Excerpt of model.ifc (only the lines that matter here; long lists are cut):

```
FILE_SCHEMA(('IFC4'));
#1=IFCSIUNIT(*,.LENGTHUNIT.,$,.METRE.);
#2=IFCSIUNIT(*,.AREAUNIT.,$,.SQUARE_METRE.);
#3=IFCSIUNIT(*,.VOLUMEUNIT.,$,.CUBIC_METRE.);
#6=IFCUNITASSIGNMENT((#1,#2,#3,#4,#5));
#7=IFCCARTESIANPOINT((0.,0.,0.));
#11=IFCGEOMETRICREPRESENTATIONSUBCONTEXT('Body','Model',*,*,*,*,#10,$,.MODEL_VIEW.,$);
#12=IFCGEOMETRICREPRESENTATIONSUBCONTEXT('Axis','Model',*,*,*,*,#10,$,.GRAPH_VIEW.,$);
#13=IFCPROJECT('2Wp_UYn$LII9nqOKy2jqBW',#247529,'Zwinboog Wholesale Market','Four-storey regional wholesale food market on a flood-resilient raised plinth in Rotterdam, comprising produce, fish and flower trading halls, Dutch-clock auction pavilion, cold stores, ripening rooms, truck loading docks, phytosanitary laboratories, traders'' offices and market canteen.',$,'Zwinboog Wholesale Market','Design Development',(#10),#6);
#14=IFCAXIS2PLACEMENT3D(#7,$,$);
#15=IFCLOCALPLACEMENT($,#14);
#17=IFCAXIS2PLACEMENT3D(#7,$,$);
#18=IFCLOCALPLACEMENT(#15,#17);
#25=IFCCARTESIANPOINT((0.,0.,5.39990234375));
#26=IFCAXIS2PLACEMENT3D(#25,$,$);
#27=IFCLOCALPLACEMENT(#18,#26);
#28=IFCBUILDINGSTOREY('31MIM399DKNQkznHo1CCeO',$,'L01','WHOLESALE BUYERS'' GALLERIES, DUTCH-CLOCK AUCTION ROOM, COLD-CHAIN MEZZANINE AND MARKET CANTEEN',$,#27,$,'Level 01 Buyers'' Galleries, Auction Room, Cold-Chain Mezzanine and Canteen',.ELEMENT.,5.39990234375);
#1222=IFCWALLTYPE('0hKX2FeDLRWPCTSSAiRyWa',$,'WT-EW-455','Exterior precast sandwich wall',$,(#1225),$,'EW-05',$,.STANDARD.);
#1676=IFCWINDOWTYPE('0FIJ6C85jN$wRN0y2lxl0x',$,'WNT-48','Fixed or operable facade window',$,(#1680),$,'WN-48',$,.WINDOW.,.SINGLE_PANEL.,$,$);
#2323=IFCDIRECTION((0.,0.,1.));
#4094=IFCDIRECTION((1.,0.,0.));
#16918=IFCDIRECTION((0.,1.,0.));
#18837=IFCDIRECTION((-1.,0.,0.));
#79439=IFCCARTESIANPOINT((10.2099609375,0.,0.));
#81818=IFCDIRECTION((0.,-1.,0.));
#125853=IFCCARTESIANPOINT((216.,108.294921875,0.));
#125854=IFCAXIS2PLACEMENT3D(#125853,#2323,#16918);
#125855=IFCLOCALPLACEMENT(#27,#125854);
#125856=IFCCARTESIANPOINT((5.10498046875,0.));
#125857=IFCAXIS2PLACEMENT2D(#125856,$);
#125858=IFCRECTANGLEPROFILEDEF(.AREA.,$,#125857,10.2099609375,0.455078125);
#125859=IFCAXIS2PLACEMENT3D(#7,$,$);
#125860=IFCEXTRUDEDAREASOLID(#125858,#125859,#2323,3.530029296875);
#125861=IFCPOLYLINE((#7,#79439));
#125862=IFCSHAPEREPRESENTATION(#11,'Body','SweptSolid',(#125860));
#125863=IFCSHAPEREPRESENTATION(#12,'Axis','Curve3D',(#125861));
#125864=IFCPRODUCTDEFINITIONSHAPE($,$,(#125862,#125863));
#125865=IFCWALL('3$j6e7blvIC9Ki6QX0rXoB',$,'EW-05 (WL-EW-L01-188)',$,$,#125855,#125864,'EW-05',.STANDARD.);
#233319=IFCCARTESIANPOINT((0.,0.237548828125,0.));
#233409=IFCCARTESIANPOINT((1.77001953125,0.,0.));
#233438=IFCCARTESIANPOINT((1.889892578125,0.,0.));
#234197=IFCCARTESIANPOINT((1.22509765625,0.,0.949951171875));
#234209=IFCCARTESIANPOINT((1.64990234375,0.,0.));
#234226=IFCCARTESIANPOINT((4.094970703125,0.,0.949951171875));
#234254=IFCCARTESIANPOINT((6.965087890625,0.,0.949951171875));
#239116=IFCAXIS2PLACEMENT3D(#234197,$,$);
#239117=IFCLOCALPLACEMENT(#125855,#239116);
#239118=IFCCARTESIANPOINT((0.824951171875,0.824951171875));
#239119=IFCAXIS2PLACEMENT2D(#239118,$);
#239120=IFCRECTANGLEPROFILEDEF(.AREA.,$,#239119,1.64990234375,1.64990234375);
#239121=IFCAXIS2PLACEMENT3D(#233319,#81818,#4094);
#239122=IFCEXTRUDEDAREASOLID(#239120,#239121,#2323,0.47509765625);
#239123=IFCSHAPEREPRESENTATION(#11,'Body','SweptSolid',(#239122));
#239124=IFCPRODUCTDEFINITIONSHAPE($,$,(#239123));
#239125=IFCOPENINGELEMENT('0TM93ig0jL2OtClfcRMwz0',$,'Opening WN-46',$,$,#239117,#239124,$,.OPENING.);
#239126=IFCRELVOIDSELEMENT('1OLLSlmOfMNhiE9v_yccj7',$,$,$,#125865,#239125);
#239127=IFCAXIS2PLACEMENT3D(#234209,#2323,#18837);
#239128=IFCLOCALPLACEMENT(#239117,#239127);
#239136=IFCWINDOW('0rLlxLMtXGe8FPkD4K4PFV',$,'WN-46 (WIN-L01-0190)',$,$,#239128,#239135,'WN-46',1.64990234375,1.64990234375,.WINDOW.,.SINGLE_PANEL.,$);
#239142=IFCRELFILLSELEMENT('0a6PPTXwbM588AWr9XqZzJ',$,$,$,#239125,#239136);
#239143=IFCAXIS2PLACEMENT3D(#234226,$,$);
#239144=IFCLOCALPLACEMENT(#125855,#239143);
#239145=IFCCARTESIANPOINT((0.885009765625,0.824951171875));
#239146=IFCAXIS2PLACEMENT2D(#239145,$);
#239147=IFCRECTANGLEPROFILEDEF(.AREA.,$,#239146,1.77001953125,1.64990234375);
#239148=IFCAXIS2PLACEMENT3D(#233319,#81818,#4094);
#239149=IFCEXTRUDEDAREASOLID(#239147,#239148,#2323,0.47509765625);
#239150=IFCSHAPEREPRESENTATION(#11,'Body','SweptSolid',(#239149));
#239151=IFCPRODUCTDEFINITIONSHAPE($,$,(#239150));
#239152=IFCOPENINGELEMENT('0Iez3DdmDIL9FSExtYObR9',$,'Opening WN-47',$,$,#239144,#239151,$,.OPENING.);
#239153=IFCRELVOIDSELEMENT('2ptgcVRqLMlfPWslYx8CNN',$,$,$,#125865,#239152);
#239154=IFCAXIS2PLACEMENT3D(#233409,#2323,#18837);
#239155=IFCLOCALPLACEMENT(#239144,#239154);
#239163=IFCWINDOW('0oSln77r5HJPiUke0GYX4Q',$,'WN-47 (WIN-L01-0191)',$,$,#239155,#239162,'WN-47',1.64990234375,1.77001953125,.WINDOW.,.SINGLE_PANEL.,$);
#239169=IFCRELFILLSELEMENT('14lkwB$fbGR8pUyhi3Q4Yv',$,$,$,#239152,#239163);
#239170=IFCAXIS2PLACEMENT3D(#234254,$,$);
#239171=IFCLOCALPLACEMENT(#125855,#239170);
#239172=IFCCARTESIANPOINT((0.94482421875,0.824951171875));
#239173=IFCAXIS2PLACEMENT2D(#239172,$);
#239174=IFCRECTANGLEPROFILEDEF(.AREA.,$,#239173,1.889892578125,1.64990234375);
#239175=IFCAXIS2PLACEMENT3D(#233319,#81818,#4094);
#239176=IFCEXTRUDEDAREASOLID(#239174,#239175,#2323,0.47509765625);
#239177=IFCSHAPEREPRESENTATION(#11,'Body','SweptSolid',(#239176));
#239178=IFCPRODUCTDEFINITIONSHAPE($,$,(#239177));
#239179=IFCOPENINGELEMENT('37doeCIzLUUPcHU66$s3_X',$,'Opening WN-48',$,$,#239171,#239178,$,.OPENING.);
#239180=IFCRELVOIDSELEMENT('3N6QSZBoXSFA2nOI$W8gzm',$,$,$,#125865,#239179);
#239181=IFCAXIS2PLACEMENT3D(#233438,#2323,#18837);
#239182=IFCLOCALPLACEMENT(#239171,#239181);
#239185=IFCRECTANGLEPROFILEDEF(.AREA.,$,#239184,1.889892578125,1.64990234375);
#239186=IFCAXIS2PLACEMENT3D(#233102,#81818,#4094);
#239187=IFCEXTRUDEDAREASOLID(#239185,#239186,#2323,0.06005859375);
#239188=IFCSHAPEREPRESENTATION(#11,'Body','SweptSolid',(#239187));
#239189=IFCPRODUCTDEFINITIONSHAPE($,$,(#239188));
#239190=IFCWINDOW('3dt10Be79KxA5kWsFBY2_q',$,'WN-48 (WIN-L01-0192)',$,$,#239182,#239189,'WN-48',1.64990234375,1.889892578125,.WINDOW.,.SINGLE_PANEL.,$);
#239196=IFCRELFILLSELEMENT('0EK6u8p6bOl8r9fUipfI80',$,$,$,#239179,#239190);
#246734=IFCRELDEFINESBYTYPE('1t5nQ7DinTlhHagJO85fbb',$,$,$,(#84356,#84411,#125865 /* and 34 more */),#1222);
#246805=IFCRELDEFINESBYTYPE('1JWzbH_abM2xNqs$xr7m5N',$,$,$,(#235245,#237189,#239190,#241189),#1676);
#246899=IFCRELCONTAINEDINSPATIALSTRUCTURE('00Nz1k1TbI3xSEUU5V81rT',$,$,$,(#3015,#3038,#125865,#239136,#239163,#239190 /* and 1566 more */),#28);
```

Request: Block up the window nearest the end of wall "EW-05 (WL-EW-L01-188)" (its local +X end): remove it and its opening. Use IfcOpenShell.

```python
import ifcopenshell
import ifcopenshell.api.feature
import ifcopenshell.api.root
import ifcopenshell.geom
import ifcopenshell.util.shape

model = ifcopenshell.open("model.ifc")
settings = ifcopenshell.geom.settings()


def volume(element):
    """Net volume in cubic metres, openings subtracted."""
    shape = ifcopenshell.geom.create_shape(settings, element)
    return ifcopenshell.util.shape.get_volume(shape.geometry)


window = model.by_guid("3dt10Be79KxA5kWsFBY2_q")
opening = window.FillsVoids[0].RelatingOpeningElement
wall = opening.VoidsElements[0].RelatingBuildingElement
before = volume(wall)

ifcopenshell.api.root.remove_product(model, product=window)
ifcopenshell.api.feature.remove_feature(model, feature=opening)

after = volume(wall)

print(f"wall volume {before:.3f} -> {after:.3f} m3")

model.write("model_edited.ifc")
```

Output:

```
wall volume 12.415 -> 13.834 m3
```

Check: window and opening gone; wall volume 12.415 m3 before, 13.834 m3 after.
